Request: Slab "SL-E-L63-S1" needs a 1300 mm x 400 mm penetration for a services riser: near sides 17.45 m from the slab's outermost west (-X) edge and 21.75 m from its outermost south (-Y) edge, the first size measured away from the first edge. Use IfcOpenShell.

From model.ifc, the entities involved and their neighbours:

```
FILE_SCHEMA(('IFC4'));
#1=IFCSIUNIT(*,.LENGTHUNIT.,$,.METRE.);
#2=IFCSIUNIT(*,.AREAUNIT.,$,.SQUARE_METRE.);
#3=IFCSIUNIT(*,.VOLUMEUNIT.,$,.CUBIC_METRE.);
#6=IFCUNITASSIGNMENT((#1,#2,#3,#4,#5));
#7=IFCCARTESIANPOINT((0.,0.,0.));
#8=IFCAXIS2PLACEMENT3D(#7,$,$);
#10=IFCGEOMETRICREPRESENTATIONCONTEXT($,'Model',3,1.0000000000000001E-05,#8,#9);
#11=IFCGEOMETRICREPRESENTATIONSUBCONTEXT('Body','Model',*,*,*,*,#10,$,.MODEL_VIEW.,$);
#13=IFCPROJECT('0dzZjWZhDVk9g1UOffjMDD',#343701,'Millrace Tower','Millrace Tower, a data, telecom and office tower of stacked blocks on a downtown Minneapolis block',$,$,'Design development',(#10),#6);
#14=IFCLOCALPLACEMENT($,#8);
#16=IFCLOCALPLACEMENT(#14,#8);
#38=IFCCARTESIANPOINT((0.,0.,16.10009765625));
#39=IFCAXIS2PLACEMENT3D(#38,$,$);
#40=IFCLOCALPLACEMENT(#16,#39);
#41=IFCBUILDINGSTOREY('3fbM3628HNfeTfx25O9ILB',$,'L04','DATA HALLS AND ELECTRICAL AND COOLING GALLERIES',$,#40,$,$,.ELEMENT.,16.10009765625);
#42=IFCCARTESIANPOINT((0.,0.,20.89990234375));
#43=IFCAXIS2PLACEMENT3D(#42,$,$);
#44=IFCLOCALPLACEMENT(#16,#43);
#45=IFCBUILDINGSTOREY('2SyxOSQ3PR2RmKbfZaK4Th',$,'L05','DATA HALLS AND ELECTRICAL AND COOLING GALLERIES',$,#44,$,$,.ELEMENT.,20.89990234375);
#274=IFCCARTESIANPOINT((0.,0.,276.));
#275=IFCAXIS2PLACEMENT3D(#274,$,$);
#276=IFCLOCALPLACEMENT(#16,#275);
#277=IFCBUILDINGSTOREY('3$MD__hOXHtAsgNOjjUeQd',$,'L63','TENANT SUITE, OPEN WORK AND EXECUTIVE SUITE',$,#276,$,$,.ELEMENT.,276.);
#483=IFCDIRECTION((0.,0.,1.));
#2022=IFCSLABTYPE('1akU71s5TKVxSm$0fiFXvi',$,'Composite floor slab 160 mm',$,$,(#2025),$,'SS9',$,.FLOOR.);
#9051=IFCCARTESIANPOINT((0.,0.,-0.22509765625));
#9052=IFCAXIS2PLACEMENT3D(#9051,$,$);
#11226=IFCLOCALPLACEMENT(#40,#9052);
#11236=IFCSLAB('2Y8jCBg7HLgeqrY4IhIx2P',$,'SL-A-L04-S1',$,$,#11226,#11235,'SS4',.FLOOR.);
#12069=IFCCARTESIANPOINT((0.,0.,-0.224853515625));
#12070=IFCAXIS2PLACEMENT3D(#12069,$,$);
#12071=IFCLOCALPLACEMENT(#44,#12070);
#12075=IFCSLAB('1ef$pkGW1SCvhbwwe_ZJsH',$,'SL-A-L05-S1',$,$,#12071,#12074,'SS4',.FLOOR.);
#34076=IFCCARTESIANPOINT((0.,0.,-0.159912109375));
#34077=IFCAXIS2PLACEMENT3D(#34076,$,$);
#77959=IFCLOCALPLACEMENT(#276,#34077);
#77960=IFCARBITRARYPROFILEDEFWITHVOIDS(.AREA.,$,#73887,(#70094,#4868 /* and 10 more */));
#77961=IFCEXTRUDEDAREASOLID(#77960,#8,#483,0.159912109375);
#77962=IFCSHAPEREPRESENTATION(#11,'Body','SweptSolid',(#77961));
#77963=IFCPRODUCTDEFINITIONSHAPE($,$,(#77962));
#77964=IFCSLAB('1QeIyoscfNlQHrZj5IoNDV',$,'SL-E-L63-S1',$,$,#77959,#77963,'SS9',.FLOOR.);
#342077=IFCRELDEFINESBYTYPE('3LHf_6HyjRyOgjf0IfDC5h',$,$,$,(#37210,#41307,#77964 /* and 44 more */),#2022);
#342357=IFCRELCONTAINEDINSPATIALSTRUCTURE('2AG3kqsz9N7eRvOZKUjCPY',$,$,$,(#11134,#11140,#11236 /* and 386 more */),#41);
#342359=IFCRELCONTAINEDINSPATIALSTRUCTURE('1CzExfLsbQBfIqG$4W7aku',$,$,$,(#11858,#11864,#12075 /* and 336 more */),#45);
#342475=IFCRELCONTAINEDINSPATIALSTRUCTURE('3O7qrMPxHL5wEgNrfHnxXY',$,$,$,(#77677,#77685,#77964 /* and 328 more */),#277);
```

```python
import numpy as np
import ifcopenshell
import ifcopenshell.api.feature
import ifcopenshell.api.geometry
import ifcopenshell.api.root
import ifcopenshell.geom
import ifcopenshell.util.placement
import ifcopenshell.util.representation
import ifcopenshell.util.shape
import ifcopenshell.util.unit

model = ifcopenshell.open("model.ifc")
unit_scale = ifcopenshell.util.unit.calculate_unit_scale(model)
settings = ifcopenshell.geom.settings()


def volume(element):
    """Net volume in cubic metres, openings subtracted."""
    shape = ifcopenshell.geom.create_shape(settings, element)
    return ifcopenshell.util.shape.get_volume(shape.geometry)


slab = model.by_id(77964)
before = volume(slab)

# Extent in the slab's own axes, in metres. The edges named are its -X and -Y sides.
slab_shape = ifcopenshell.geom.create_shape(settings, slab)
vertices = ifcopenshell.util.shape.get_vertices(slab_shape.geometry)
x_min, y_min, bottom = vertices.min(axis=0)
top = vertices[:, 2].max()

opening = ifcopenshell.api.root.create_entity(model, ifc_class="IfcOpeningElement", name="Services riser opening", predefined_type="OPENING")
context = ifcopenshell.util.representation.get_context(model, "Model", "Body", "MODEL_VIEW")
width, depth = 1.3, 0.4
outline = [(0.0, 0.0), (width, 0.0), (width, depth), (0.0, depth), (0.0, 0.0)]
# Overshoot both faces by 50 mm so the cut is clean.
shape = ifcopenshell.api.geometry.add_slab_representation(
    model, context=context, depth=top - bottom + 0.1, polyline=outline
)
ifcopenshell.api.geometry.assign_representation(model, product=opening, representation=shape)

matrix = ifcopenshell.util.placement.get_local_placement(slab.ObjectPlacement)
matrix[:, 3] = matrix @ np.append(np.array([x_min + 17.45, y_min + 21.75, bottom - 0.05]) / unit_scale, 1.0)
ifcopenshell.api.geometry.edit_object_placement(model, product=opening, matrix=matrix, is_si=False)
ifcopenshell.api.feature.add_feature(model, feature=opening, element=slab)

after = volume(slab)

print(f"slab volume {before:.3f} -> {after:.3f} m3")

model.write("model_rev.ifc")
```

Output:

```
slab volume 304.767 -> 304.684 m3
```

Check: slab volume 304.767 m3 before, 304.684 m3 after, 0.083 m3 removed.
